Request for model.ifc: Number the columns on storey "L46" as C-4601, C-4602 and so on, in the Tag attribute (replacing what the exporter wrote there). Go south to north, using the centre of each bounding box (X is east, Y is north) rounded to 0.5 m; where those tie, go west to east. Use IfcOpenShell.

First a look at what the model holds.

```python
import ifcopenshell
import ifcopenshell.util.element
import ifcopenshell.util.placement

model = ifcopenshell.open("model.ifc")
print(model.schema)
storey = next(s for s in model.by_type("IfcBuildingStorey") if s.Name == "L46")
columns = [e for e in ifcopenshell.util.element.get_decomposition(storey) if e.is_a("IfcColumn")]
for e in sorted(columns, key=lambda e: e.id()):
    origin = ifcopenshell.util.placement.get_local_placement(e.ObjectPlacement)[:3, 3]
    print(e.id(), e.Tag, e.Name, origin.round(2) + 0.0, sep=" | ")
```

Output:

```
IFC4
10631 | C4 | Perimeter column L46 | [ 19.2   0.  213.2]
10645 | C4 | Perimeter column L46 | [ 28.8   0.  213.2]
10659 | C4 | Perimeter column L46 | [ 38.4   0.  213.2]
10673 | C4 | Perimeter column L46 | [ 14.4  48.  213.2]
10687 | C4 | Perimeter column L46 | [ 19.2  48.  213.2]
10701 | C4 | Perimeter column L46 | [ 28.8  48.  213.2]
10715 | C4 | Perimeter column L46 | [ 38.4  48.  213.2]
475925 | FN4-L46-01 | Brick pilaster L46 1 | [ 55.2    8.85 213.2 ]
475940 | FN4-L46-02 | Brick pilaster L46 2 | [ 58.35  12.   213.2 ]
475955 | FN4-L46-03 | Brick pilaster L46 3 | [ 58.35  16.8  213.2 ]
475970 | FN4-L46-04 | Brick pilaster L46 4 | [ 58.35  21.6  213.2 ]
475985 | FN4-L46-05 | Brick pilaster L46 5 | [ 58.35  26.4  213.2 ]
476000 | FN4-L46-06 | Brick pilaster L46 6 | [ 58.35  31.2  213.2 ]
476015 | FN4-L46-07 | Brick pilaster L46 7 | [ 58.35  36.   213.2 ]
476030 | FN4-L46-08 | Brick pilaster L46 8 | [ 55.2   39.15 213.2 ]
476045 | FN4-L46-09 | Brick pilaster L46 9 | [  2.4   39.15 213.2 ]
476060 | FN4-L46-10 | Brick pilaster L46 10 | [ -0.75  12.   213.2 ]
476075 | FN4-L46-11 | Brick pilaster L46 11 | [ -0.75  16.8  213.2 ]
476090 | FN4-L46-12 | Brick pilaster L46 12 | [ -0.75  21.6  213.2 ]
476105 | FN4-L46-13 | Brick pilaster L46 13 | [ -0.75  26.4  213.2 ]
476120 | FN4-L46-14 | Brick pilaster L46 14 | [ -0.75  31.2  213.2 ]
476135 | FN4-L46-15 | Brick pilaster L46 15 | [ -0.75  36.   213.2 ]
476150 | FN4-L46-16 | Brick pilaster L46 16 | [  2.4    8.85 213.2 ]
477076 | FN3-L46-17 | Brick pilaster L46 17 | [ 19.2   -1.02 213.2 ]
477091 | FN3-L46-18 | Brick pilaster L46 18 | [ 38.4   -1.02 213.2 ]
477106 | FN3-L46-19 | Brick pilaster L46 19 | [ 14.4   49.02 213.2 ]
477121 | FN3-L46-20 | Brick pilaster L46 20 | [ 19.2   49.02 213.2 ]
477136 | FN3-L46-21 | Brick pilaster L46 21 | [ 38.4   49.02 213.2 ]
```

```python
import ifcopenshell
import ifcopenshell.geom
import ifcopenshell.util.element
import ifcopenshell.util.shape

model = ifcopenshell.open("model.ifc")
settings = ifcopenshell.geom.settings()
settings.set("use-world-coords", True)


def centre(element):
    shape = ifcopenshell.geom.create_shape(settings, element)
    return ifcopenshell.util.shape.get_bbox_centroid(shape.geometry)


storey = next(s for s in model.by_type("IfcBuildingStorey") if s.Name == "L46")
columns = [e for e in ifcopenshell.util.element.get_decomposition(storey) if e.is_a("IfcColumn")]

# Insertion points can sit at a corner or the storey origin, so sort by the geometry (in metres).
centres = {e: centre(e) for e in columns}
columns.sort(key=lambda e: (round(centres[e][1] / 0.5), centres[e][0]))

for i, e in enumerate(columns, start=1):
    number = f"C-46{i:02d}"
    e.Tag = number
    print(e.id(), number)

model.write("model_updated.ifc")
```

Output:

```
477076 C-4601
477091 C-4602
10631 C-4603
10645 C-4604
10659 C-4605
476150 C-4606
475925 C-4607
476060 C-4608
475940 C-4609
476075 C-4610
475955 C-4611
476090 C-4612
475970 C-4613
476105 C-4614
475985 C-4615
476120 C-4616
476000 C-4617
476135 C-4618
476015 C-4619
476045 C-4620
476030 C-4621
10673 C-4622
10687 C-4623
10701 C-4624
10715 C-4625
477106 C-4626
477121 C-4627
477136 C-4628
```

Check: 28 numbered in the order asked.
